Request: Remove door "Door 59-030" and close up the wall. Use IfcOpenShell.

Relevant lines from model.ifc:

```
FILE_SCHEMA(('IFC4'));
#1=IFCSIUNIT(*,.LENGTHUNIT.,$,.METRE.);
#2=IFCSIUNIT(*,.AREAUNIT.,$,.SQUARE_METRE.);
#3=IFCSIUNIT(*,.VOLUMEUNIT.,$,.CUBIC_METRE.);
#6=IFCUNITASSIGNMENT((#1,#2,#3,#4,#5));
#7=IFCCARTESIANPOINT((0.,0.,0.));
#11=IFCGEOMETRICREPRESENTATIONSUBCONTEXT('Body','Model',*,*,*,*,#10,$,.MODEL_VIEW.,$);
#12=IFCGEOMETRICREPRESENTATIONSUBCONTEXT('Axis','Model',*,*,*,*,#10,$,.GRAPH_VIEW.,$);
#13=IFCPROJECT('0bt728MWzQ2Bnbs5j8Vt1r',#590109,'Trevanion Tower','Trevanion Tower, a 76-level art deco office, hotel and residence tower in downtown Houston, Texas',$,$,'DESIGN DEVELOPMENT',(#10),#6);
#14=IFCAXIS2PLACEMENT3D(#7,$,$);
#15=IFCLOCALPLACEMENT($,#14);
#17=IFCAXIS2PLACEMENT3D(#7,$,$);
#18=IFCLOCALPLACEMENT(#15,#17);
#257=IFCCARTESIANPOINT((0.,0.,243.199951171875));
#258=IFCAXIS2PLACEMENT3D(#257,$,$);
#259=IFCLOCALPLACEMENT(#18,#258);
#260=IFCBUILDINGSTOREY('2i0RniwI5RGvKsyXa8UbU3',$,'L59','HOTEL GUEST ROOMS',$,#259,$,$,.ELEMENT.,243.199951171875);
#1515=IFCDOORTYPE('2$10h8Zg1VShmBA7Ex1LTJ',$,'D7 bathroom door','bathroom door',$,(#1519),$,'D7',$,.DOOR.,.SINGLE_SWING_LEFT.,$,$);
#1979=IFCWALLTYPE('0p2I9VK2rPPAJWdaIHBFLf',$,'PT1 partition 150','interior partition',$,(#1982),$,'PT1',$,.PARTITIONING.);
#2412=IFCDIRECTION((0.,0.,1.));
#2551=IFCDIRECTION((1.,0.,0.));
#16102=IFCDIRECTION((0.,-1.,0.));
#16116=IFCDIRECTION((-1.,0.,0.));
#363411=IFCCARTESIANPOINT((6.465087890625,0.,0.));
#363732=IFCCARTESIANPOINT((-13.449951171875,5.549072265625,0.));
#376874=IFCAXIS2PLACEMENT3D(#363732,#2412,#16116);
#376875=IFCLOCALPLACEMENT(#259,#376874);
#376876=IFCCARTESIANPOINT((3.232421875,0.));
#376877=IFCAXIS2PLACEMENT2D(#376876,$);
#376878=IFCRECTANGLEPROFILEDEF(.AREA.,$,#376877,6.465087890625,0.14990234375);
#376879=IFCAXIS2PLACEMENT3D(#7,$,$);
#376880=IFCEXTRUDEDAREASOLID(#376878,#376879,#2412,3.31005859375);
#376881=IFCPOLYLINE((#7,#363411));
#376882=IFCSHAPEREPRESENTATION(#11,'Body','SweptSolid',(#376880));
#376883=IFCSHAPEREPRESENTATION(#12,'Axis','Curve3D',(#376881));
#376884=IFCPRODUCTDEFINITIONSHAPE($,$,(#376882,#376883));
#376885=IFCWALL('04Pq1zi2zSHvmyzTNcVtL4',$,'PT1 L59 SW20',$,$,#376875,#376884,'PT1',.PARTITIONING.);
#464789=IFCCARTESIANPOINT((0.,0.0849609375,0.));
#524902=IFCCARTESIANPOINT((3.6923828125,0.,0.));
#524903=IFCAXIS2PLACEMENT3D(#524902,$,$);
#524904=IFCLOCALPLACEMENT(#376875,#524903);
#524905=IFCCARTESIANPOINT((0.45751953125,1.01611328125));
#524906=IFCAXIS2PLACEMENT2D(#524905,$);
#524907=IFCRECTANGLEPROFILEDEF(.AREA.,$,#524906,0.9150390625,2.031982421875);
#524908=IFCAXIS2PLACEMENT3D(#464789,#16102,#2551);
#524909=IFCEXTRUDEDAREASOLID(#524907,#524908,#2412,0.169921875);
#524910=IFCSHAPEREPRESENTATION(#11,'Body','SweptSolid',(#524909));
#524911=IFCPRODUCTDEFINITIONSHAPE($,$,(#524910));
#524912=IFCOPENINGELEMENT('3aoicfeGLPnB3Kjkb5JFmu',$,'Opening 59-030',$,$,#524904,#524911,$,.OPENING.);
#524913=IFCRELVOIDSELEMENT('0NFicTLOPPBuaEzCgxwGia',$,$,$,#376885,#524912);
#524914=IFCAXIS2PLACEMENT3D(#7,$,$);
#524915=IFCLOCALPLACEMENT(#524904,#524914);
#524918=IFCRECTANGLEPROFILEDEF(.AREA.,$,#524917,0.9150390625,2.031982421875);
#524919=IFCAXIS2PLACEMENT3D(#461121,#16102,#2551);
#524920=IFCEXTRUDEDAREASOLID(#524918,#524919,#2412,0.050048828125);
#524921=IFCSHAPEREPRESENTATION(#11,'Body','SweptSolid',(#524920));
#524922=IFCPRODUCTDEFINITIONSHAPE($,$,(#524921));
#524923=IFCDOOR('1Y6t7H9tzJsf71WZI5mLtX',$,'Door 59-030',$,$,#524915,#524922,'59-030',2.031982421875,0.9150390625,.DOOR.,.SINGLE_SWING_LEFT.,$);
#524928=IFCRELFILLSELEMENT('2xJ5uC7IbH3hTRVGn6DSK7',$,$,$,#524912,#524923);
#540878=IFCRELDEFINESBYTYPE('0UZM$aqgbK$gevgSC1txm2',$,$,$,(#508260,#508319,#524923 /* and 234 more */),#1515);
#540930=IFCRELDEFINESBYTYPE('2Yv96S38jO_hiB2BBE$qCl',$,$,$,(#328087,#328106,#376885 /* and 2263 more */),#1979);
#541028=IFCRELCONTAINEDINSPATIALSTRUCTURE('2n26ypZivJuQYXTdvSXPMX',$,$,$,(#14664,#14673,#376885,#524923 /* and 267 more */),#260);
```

```python
import ifcopenshell
import ifcopenshell.api.feature
import ifcopenshell.api.root
import ifcopenshell.geom
import ifcopenshell.util.shape

model = ifcopenshell.open("model.ifc")
settings = ifcopenshell.geom.settings()


def volume(element):
    """Net volume in cubic metres, openings subtracted."""
    shape = ifcopenshell.geom.create_shape(settings, element)
    return ifcopenshell.util.shape.get_volume(shape.geometry)


door = model.by_guid("1Y6t7H9tzJsf71WZI5mLtX")
opening = door.FillsVoids[0].RelatingOpeningElement
wall = opening.VoidsElements[0].RelatingBuildingElement
before = volume(wall)

ifcopenshell.api.root.remove_product(model, product=door)
ifcopenshell.api.feature.remove_feature(model, feature=opening)

after = volume(wall)

print(f"wall volume {before:.3f} -> {after:.3f} m3")

model.write("model_edited.ifc")
```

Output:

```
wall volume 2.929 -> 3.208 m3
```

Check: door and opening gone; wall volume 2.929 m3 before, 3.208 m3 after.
